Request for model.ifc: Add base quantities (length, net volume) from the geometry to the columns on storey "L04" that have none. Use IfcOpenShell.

First a look at what the model holds.

```python
import ifcopenshell
import ifcopenshell.util.element
import ifcopenshell.util.unit

model = ifcopenshell.open("model.ifc")
print(model.schema)
for unit_type in ("LENGTHUNIT", "AREAUNIT", "VOLUMEUNIT"):
    print(unit_type, ifcopenshell.util.unit.calculate_unit_scale(model, unit_type))
storey = next(s for s in model.by_type("IfcBuildingStorey") if s.Name == "L04")
columns = [e for e in ifcopenshell.util.element.get_decomposition(storey) if e.is_a("IfcColumn")]
for e in sorted(columns, key=lambda e: e.id()):
    print(e.id(), e.is_a(), e.Name, list(ifcopenshell.util.element.get_psets(e, qtos_only=True)), sep=" | ")
```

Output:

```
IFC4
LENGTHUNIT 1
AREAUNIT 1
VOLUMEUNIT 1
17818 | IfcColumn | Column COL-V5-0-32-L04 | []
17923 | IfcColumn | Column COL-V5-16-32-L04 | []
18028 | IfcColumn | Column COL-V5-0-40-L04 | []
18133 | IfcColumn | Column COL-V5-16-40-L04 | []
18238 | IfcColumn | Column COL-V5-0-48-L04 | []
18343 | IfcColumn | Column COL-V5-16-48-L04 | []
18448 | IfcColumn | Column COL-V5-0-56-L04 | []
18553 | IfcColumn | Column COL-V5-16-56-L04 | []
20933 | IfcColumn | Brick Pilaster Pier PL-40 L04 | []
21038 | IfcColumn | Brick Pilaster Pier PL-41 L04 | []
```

```python
import ifcopenshell
import ifcopenshell.api.pset
import ifcopenshell.geom
import ifcopenshell.util.element
import ifcopenshell.util.shape
import ifcopenshell.util.unit

model = ifcopenshell.open("model.ifc")
unit_scale = ifcopenshell.util.unit.calculate_unit_scale(model)
volume_scale = ifcopenshell.util.unit.calculate_unit_scale(model, "VOLUMEUNIT")
settings = ifcopenshell.geom.settings()

storey = next(s for s in model.by_type("IfcBuildingStorey") if s.Name == "L04")
columns = [e for e in ifcopenshell.util.element.get_decomposition(storey) if e.is_a("IfcColumn")]

for e in sorted(columns, key=lambda e: e.id()):
    if ifcopenshell.util.element.get_psets(e, qtos_only=True, should_inherit=False):
        continue
    # Geometry comes back in metres, in the element's own axes.
    shape = ifcopenshell.geom.create_shape(settings, e)
    values = {
        "Length": ifcopenshell.util.shape.get_z(shape.geometry) / unit_scale,
        "NetVolume": ifcopenshell.util.shape.get_volume(shape.geometry) / volume_scale,
    }
    qto = ifcopenshell.api.pset.add_qto(model, product=e, name="Qto_ColumnBaseQuantities")
    ifcopenshell.api.pset.edit_qto(model, qto=qto, properties=values)
    print(e.id(), {k: round(v, 3) for k, v in values.items()})

model.write("model_edited.ifc")
```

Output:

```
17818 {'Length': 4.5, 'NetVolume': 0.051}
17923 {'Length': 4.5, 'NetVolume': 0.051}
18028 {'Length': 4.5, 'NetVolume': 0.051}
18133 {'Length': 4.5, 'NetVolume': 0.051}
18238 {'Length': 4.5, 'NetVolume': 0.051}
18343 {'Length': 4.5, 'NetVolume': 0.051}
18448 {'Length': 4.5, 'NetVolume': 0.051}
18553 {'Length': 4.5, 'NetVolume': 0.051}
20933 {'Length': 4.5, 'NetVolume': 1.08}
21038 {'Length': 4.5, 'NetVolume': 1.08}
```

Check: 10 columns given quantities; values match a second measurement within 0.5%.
